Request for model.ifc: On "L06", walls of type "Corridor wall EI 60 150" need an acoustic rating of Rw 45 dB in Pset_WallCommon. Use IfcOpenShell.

First a look at what the model holds.

```python
import ifcopenshell
import ifcopenshell.util.element

model = ifcopenshell.open("model.ifc")
print(model.schema)
storey = next(s for s in model.by_type("IfcBuildingStorey") if s.Name == "L06")
walls = [e for e in ifcopenshell.util.element.get_decomposition(storey) if e.is_a("IfcWall")]
seen = {}
for e in walls:
    element_type = ifcopenshell.util.element.get_type(e)
    key = (element_type.Name if element_type != e and element_type else None, ifcopenshell.util.element.get_pset(e, "Pset_WallCommon", "AcousticRating"))
    seen[key] = seen.get(key, 0) + 1
for (name, value), count in sorted(seen.items(), key=str):
    print(count, "x", name, "|", value)
```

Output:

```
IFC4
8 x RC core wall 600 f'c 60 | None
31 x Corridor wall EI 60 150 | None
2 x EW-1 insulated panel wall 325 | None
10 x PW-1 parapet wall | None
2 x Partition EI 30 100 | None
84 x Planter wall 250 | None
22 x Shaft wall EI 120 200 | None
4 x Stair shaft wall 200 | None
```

```python
import ifcopenshell
import ifcopenshell.api.pset
import ifcopenshell.util.element

model = ifcopenshell.open("model.ifc")

storey = next(s for s in model.by_type("IfcBuildingStorey") if s.Name == "L06")
walls = [e for e in ifcopenshell.util.element.get_decomposition(storey) if e.is_a("IfcWall")]

count = 0
for e in walls:
    element_type = ifcopenshell.util.element.get_type(e)
    if element_type in (None, e) or element_type.Name != "Corridor wall EI 60 150":
        continue
    found = ifcopenshell.util.element.get_pset(e, "Pset_WallCommon", should_inherit=False)
    if found:
        pset = model.by_id(found["id"])
        if len(ifcopenshell.util.element.get_elements_by_pset(pset)) > 1:
            pset = ifcopenshell.api.pset.unshare_pset(model, products=[e], pset=pset)[0]
    else:
        pset = ifcopenshell.api.pset.add_pset(model, product=e, name="Pset_WallCommon")
    ifcopenshell.api.pset.edit_pset(model, pset=pset, properties={"AcousticRating": "Rw 45 dB"})
    count += 1

print(count, "walls updated")

model.write("model-out.ifc")
```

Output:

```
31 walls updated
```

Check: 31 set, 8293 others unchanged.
